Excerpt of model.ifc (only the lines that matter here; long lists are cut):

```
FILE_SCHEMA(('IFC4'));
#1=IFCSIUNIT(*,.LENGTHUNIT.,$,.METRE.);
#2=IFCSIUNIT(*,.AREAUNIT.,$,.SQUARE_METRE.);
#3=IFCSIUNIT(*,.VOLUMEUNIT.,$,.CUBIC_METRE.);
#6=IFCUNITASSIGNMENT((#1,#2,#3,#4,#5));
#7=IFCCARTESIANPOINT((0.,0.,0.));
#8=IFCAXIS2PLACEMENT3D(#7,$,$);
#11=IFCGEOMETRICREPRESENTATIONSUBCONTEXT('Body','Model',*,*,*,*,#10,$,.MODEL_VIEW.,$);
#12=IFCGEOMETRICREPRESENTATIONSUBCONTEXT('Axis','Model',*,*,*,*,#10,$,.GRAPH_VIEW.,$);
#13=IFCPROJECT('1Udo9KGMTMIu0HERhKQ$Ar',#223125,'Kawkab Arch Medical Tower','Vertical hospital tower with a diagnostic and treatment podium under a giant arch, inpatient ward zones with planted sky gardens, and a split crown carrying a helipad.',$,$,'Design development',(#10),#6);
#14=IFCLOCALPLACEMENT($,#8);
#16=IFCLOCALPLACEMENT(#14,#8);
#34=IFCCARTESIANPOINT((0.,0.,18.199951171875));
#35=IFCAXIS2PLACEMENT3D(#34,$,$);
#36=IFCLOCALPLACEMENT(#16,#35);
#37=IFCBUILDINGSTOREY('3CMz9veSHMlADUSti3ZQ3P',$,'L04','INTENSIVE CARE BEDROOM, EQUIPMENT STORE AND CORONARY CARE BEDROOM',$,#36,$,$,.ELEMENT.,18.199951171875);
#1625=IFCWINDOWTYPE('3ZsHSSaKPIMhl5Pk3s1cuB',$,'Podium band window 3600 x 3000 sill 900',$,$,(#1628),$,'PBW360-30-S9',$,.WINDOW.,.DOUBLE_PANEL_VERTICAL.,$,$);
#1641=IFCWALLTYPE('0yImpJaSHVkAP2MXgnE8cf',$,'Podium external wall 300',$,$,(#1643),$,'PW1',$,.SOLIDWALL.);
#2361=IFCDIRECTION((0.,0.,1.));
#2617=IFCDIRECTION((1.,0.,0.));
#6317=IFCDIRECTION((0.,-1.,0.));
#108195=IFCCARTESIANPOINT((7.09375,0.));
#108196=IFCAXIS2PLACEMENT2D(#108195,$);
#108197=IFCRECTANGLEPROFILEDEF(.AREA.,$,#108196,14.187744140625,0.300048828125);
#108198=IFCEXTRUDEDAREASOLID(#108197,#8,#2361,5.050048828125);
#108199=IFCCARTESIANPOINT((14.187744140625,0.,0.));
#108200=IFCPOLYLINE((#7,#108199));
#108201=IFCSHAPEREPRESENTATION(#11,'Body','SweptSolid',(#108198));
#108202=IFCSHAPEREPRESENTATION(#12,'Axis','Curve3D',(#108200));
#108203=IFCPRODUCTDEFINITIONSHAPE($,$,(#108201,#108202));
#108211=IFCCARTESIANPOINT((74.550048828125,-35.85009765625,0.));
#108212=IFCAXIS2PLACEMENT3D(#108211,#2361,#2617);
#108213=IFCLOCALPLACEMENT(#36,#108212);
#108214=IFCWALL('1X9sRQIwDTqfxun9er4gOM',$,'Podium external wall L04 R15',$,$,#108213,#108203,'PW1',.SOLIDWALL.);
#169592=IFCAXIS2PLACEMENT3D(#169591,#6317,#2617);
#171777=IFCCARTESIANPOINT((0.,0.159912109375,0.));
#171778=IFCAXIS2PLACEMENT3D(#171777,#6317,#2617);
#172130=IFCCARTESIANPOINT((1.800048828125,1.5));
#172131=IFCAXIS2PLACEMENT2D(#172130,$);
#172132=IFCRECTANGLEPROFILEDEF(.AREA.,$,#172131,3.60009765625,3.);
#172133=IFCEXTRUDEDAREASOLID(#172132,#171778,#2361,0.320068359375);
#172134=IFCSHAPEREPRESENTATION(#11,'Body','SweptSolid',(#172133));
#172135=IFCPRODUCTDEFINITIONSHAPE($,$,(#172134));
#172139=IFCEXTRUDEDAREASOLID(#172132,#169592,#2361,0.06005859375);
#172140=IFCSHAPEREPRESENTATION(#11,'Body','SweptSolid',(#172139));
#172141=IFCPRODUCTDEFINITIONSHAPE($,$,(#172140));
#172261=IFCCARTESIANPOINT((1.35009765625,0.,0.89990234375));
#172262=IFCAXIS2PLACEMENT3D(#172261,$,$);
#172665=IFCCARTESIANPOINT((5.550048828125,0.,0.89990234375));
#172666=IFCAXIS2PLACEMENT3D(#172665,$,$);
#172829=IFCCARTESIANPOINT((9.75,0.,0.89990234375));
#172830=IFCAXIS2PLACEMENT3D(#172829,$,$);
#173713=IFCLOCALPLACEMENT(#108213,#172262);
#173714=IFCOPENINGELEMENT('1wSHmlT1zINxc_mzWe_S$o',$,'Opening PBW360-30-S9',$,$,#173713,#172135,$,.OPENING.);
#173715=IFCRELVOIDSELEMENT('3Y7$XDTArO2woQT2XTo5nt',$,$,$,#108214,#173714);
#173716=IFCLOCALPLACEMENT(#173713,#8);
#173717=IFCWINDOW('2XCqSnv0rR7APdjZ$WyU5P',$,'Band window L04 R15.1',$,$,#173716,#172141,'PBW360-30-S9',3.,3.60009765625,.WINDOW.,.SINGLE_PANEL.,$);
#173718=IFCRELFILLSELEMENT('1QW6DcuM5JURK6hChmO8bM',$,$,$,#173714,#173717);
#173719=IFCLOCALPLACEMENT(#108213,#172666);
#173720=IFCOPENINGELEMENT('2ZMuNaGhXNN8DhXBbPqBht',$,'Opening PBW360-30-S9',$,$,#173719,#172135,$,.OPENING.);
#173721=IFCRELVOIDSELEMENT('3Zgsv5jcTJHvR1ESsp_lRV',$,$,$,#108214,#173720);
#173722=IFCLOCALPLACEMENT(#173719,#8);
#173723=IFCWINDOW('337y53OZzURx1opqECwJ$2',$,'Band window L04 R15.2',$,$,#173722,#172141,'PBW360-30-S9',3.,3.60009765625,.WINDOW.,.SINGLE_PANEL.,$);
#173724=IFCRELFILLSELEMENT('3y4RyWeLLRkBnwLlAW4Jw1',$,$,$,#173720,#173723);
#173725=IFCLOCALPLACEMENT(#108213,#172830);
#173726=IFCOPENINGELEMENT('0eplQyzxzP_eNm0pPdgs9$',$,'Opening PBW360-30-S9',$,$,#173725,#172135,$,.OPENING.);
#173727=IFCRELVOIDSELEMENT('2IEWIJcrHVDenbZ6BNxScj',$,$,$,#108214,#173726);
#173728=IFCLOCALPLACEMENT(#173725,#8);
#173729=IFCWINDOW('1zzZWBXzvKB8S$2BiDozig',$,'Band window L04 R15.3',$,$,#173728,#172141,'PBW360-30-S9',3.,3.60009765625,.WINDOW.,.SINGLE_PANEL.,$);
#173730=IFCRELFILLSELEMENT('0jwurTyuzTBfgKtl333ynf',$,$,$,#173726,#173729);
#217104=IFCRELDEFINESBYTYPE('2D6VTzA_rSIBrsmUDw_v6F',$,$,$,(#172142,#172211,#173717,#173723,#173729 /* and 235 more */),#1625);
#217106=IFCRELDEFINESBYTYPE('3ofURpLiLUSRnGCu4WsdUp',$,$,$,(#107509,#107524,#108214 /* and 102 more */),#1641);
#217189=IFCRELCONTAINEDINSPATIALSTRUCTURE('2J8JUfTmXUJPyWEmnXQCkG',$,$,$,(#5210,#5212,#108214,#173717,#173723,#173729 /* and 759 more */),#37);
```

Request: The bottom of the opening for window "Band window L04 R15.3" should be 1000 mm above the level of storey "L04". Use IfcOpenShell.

```python
import numpy as np
import ifcopenshell
import ifcopenshell.api.geometry
import ifcopenshell.geom
import ifcopenshell.util.element
import ifcopenshell.util.placement
import ifcopenshell.util.shape
import ifcopenshell.util.unit

model = ifcopenshell.open("model.ifc")
unit_scale = ifcopenshell.util.unit.calculate_unit_scale(model)

window = model.by_guid("1zzZWBXzvKB8S$2BiDozig")
opening = window.FillsVoids[0].RelatingOpeningElement
storey = ifcopenshell.util.element.get_container(window, ifc_class="IfcBuildingStorey")
level = ifcopenshell.util.placement.get_local_placement(storey.ObjectPlacement)[2, 3]

# The opening's origin need not be at the sill, so measure its lowest point.
shape = ifcopenshell.geom.create_shape(ifcopenshell.geom.settings(), opening)
bottom = ifcopenshell.util.shape.get_shape_bottom_elevation(shape, shape.geometry) / unit_scale
dz = level + 1 / unit_scale - bottom

shift = np.array([0.0, 0.0, dz])
# The window is placed relative to its opening, so it follows when the opening moves.
matrix = ifcopenshell.util.placement.get_local_placement(opening.ObjectPlacement)
matrix[:3, 3] += shift
ifcopenshell.api.geometry.edit_object_placement(
    model, product=opening, matrix=matrix, is_si=False, should_transform_children=True
)

print(f"moved by {dz * unit_scale:+.3f} m")

model.write("model-out.ifc")
```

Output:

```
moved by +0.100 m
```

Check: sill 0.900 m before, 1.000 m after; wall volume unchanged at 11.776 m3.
